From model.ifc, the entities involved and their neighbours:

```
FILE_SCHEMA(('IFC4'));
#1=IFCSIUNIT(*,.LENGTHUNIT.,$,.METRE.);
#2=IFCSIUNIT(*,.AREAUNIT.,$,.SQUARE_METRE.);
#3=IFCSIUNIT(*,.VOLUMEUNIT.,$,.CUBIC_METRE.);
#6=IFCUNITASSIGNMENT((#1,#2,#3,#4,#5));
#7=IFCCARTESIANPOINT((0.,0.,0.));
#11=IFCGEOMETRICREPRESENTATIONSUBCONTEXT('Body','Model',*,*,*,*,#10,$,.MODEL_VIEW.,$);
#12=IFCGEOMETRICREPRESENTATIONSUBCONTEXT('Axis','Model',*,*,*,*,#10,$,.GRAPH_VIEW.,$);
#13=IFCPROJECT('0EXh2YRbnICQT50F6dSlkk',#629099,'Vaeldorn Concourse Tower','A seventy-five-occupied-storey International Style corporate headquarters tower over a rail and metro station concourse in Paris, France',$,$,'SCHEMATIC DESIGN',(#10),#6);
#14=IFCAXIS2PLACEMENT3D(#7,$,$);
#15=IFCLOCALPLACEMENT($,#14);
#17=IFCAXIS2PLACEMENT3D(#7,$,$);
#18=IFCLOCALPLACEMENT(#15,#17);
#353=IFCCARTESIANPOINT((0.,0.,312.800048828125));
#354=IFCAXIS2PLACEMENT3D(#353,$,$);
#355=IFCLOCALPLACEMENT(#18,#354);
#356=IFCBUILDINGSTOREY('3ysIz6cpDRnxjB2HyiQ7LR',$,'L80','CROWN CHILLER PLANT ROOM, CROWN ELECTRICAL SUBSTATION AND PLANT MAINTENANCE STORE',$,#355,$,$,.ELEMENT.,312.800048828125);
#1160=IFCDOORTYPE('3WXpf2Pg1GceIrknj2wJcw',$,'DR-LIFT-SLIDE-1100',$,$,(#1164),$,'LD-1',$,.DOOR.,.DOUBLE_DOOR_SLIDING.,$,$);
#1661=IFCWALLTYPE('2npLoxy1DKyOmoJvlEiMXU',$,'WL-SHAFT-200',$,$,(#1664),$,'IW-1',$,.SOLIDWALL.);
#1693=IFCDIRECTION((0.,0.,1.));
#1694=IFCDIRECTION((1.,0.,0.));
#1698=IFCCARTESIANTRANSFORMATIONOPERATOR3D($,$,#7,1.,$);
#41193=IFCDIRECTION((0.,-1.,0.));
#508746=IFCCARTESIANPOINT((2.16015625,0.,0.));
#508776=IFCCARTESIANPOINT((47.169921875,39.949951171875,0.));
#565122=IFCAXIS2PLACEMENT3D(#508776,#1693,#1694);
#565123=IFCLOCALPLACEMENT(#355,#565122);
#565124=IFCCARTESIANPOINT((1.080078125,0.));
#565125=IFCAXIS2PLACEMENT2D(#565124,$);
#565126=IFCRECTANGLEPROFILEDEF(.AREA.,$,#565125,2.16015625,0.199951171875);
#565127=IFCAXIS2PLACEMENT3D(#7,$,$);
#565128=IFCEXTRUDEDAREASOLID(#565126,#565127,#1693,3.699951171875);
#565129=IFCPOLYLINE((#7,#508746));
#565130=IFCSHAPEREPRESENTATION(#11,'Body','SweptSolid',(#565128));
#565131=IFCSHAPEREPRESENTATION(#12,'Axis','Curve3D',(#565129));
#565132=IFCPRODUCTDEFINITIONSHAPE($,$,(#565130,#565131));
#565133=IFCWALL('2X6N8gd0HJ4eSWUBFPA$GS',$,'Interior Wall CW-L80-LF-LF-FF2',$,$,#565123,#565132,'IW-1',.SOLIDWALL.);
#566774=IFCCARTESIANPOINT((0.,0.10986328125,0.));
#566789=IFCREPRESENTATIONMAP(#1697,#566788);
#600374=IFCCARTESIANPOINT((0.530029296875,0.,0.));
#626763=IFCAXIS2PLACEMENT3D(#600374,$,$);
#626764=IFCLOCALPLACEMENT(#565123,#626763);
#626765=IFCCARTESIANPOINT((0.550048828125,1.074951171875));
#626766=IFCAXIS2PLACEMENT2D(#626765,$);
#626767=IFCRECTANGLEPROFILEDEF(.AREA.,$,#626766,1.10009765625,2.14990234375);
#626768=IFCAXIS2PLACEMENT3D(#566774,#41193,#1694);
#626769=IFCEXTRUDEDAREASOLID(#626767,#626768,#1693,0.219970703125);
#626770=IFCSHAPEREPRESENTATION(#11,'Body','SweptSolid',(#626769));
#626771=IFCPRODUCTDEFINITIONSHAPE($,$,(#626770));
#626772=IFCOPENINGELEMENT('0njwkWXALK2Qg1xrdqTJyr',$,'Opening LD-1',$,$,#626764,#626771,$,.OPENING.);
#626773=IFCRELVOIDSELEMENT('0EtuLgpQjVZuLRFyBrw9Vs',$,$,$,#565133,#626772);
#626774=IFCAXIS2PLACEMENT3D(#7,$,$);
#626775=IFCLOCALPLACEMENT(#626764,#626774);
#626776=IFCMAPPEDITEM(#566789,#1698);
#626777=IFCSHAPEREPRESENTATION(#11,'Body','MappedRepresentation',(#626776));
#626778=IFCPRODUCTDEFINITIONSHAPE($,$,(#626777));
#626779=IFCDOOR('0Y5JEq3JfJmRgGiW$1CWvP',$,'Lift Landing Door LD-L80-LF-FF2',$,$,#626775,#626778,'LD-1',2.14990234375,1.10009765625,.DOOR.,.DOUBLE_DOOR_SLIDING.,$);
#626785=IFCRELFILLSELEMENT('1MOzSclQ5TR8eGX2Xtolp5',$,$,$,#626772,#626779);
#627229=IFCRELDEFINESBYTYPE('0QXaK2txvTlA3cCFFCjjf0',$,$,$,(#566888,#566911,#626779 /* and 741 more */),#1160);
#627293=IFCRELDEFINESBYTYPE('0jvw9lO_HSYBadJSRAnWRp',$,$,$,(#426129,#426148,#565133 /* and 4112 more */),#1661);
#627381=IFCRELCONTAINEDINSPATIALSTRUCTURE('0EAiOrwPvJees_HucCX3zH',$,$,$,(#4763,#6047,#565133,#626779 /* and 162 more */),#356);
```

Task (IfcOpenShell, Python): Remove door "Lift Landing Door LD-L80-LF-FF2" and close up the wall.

```python
import ifcopenshell
import ifcopenshell.api.feature
import ifcopenshell.api.root
import ifcopenshell.geom
import ifcopenshell.util.shape

model = ifcopenshell.open("model.ifc")
settings = ifcopenshell.geom.settings()


def volume(element):
    """Net volume in cubic metres, openings subtracted."""
    shape = ifcopenshell.geom.create_shape(settings, element)
    return ifcopenshell.util.shape.get_volume(shape.geometry)


door = model.by_guid("0Y5JEq3JfJmRgGiW$1CWvP")
opening = door.FillsVoids[0].RelatingOpeningElement
wall = opening.VoidsElements[0].RelatingBuildingElement
before = volume(wall)

ifcopenshell.api.root.remove_product(model, product=door)
ifcopenshell.api.feature.remove_feature(model, feature=opening)

after = volume(wall)

print(f"wall volume {before:.3f} -> {after:.3f} m3")

model.write("model-out.ifc")
```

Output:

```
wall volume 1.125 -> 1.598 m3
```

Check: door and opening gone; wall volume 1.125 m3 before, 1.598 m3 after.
